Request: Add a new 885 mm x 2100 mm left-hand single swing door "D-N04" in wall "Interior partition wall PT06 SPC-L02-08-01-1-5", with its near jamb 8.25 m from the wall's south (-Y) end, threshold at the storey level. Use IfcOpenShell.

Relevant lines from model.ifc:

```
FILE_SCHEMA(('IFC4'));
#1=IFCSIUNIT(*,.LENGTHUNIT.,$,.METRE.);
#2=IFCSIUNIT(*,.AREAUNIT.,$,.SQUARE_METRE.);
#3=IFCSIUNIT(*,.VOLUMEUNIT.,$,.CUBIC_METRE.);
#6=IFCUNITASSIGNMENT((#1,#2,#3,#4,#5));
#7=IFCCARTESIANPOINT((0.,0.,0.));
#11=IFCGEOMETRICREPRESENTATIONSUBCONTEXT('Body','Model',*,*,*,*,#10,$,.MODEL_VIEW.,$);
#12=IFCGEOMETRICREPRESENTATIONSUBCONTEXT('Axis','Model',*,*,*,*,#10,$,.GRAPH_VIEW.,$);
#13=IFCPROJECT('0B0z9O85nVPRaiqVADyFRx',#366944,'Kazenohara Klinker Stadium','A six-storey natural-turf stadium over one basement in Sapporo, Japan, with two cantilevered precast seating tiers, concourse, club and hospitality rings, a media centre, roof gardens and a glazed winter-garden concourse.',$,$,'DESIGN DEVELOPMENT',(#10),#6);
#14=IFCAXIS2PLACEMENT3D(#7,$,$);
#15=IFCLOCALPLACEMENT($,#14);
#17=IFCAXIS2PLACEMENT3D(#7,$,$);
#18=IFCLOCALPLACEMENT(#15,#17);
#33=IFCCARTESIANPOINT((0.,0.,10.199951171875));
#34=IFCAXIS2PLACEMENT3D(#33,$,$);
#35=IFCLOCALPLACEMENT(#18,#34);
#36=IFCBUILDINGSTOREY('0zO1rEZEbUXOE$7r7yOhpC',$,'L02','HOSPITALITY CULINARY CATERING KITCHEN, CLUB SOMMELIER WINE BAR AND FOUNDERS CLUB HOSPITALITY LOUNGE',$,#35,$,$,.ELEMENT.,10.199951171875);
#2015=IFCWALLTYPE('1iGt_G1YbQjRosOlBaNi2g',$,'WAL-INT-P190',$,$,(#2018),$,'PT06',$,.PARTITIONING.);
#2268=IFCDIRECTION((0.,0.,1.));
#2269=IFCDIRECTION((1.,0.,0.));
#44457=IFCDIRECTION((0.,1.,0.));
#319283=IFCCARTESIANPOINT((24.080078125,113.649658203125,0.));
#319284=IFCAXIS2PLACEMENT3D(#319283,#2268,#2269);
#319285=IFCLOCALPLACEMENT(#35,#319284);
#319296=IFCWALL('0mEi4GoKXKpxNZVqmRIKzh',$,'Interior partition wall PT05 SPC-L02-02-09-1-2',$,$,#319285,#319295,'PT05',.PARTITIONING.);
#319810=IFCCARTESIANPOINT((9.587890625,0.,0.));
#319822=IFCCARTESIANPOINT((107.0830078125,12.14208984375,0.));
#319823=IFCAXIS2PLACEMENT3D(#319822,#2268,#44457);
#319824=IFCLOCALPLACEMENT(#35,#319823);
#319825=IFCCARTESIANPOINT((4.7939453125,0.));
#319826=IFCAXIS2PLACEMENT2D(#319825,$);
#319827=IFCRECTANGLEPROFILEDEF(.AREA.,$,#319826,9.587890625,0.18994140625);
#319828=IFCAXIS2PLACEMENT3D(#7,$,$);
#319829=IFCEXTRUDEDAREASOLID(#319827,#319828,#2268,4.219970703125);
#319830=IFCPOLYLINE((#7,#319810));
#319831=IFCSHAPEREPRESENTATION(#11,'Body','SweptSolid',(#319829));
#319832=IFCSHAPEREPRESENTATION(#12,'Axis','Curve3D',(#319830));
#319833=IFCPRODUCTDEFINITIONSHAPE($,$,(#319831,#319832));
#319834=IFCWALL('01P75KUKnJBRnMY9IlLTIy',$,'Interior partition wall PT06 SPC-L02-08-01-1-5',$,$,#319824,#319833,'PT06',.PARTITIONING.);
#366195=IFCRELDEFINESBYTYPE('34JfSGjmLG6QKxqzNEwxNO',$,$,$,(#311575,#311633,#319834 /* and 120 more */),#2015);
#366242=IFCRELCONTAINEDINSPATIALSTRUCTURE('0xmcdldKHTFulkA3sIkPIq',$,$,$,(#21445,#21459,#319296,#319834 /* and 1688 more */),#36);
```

```python
import numpy as np
import ifcopenshell
import ifcopenshell.api.feature
import ifcopenshell.api.geometry
import ifcopenshell.api.root
import ifcopenshell.api.spatial
import ifcopenshell.geom
import ifcopenshell.util.element
import ifcopenshell.util.placement
import ifcopenshell.util.representation
import ifcopenshell.util.shape
import ifcopenshell.util.unit

model = ifcopenshell.open("model.ifc")
unit_scale = ifcopenshell.util.unit.calculate_unit_scale(model)
settings = ifcopenshell.geom.settings()


def volume(element):
    """Net volume in cubic metres, openings subtracted."""
    shape = ifcopenshell.geom.create_shape(settings, element)
    return ifcopenshell.util.shape.get_volume(shape.geometry)


wall = model.by_id(319834)
storey = ifcopenshell.util.element.get_container(wall, ifc_class="IfcBuildingStorey")
context = ifcopenshell.util.representation.get_context(model, "Model", "Body", "MODEL_VIEW")
before = volume(wall)

width, height, from_end, sill = 0.885, 2.1, 8.25, 0.0  # metres

# The wall runs along its own X axis, and the end named is its -X end.
wall_shape = ifcopenshell.geom.create_shape(settings, wall)
x, y, z = ifcopenshell.util.shape.get_vertices(wall_shape.geometry).T
start = x.min() + from_end
face, thickness = float(y.min()), float(y.max() - y.min())
wall_matrix = ifcopenshell.util.placement.get_local_placement(wall.ObjectPlacement)
level = ifcopenshell.util.placement.get_local_placement(storey.ObjectPlacement)[2, 3]


def in_wall(x, y):
    """Placement at x, y metres in the wall's axes, at sill height."""
    matrix = wall_matrix.copy()
    matrix[:, 3] = wall_matrix @ np.array([x / unit_scale, y / unit_scale, 0.0, 1.0])
    matrix[2, 3] = level + sill / unit_scale
    return matrix


# Opening: a box that overshoots both wall faces by 50 mm.
opening = ifcopenshell.api.root.create_entity(model, ifc_class="IfcOpeningElement", predefined_type="OPENING")
box = ifcopenshell.api.geometry.add_wall_representation(
    model, context=context, length=width, height=height, thickness=thickness + 0.1
)
ifcopenshell.api.geometry.assign_representation(model, product=opening, representation=box)
ifcopenshell.api.geometry.edit_object_placement(model, product=opening, matrix=in_wall(start, face - 0.05), is_si=False)
ifcopenshell.api.feature.add_feature(model, feature=opening, element=wall)

door = ifcopenshell.api.root.create_entity(model, ifc_class="IfcDoor", name="D-N04", predefined_type="DOOR")
door.OverallWidth, door.OverallHeight = width / unit_scale, height / unit_scale
door.OperationType = "SINGLE_SWING_LEFT"
body = ifcopenshell.api.geometry.add_door_representation(
    model,
    context=context,
    overall_width=door.OverallWidth,
    overall_height=door.OverallHeight,
    operation_type="SINGLE_SWING_LEFT",
    lining_properties={"LiningDepth": thickness / unit_scale, "ThresholdDepth": thickness / unit_scale},
)
ifcopenshell.api.geometry.assign_representation(model, product=door, representation=body)
ifcopenshell.api.spatial.assign_container(model, products=[door], relating_structure=storey)
ifcopenshell.api.feature.add_filling(model, opening=opening, element=door)

# The lining spans the wall, so the door starts at the wall face.
ifcopenshell.api.geometry.edit_object_placement(model, product=door, matrix=in_wall(start, face), is_si=False)

after = volume(wall)

print(f"wall volume {before:.3f} -> {after:.3f} m3")

model.write("model_updated.ifc")
```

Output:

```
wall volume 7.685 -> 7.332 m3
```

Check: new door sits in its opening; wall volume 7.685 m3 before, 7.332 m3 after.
